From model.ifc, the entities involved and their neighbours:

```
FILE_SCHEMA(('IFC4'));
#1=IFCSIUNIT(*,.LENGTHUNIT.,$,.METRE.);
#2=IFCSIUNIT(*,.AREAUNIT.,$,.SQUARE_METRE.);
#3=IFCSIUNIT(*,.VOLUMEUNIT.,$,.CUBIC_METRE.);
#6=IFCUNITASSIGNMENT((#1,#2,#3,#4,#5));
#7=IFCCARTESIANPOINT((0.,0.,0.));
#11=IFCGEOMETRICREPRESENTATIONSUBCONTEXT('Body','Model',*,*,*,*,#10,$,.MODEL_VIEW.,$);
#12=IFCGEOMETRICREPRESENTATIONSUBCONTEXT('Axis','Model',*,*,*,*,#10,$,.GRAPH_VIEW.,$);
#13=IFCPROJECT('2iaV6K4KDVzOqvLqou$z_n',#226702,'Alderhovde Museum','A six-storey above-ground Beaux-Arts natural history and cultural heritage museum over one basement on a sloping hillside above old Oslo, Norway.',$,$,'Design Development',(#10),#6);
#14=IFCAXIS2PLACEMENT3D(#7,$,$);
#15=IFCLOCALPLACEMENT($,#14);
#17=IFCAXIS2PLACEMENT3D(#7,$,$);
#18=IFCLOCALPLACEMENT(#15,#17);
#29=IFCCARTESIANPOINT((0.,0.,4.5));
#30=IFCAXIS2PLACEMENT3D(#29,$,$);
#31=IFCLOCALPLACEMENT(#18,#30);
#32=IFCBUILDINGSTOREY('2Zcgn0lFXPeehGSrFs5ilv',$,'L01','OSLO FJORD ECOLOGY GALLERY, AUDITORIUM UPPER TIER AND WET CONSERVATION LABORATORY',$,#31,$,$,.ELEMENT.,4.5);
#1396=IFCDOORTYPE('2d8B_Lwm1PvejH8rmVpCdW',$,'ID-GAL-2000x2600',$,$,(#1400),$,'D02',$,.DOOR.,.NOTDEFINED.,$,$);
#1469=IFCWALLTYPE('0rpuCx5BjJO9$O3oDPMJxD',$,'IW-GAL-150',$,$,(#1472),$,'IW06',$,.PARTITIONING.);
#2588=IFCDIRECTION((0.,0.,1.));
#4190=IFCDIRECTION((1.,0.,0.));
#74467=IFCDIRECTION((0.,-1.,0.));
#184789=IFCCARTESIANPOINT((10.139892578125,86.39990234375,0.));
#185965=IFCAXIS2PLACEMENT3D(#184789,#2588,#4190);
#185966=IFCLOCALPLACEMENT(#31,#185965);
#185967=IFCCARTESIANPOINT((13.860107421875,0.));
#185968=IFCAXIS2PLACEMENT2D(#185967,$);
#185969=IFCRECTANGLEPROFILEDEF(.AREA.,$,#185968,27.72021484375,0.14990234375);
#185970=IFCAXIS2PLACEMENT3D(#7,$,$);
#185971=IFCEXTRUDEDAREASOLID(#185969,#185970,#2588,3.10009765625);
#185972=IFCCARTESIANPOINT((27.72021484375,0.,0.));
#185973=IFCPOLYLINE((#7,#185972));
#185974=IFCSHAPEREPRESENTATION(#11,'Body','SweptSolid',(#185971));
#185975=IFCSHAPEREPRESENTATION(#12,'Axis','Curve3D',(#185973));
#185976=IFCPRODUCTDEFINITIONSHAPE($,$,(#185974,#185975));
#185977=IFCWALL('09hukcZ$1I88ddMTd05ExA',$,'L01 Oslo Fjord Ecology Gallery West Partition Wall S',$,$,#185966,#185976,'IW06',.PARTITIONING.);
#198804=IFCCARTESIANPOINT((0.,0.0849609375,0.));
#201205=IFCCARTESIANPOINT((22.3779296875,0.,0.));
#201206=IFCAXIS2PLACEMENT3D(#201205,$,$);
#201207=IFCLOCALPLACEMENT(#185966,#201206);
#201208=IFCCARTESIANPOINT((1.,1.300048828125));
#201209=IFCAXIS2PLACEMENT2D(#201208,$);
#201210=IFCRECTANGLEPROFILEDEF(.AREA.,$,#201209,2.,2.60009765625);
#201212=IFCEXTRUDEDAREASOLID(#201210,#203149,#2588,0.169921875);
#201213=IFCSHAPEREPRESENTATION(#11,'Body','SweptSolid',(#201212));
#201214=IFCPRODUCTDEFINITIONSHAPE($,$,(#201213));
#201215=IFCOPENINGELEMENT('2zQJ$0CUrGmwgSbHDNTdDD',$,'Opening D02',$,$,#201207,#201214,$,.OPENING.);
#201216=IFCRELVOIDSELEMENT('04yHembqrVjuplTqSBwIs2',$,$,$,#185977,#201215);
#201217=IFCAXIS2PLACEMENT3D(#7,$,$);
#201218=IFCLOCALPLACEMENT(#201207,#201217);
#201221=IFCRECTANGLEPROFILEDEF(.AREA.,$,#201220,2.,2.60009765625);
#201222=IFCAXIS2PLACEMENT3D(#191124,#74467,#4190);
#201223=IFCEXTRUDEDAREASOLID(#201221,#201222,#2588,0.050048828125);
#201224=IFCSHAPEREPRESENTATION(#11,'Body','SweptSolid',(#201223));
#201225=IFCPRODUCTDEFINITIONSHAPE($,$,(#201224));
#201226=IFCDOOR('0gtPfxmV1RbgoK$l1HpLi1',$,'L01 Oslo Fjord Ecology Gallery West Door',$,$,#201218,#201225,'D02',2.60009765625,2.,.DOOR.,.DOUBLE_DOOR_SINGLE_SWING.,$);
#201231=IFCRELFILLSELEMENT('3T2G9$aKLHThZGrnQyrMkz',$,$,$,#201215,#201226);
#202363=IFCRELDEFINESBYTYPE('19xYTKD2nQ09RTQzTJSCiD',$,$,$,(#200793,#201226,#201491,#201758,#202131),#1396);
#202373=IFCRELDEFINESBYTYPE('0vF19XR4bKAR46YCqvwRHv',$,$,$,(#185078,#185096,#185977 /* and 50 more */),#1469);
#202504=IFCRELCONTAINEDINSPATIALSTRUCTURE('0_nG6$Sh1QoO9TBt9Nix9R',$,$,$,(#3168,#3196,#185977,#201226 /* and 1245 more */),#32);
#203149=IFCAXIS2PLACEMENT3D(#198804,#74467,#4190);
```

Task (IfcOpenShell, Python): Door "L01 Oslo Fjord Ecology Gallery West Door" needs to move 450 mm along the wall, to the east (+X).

```python
import ifcopenshell
import ifcopenshell.api.geometry
import ifcopenshell.util.placement

model = ifcopenshell.open("model.ifc")

door = model.by_guid("0gtPfxmV1RbgoK$l1HpLi1")
opening = door.FillsVoids[0].RelatingOpeningElement
wall = opening.VoidsElements[0].RelatingBuildingElement

wall_matrix = ifcopenshell.util.placement.get_local_placement(wall.ObjectPlacement)
shift = wall_matrix[:3, 0] * 0.45
before = ifcopenshell.util.placement.get_local_placement(door.ObjectPlacement)[:3, 3].copy()

# The door is placed relative to its opening, so it follows when the opening moves.
matrix = ifcopenshell.util.placement.get_local_placement(opening.ObjectPlacement)
matrix[:3, 3] += shift
ifcopenshell.api.geometry.edit_object_placement(
    model, product=opening, matrix=matrix, is_si=False, should_transform_children=True
)

after = ifcopenshell.util.placement.get_local_placement(door.ObjectPlacement)[:3, 3]
print("door moved by", (after - before).round(3) + 0.0)

model.write("model-out.ifc")
```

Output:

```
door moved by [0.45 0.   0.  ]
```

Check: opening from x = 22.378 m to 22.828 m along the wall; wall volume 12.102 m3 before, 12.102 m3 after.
